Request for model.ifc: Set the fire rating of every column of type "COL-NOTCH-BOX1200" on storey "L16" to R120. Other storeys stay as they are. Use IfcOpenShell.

First a look at what the model holds.

```python
import ifcopenshell
import ifcopenshell.util.element

model = ifcopenshell.open("model.ifc")
print(model.schema)
storey = next(s for s in model.by_type("IfcBuildingStorey") if s.Name == "L16")
columns = [e for e in ifcopenshell.util.element.get_decomposition(storey) if e.is_a("IfcColumn")]
seen = {}
for e in columns:
    element_type = ifcopenshell.util.element.get_type(e)
    key = (element_type.Name if element_type != e and element_type else None, ifcopenshell.util.element.get_pset(e, "Pset_ColumnCommon", "FireRating"))
    seen[key] = seen.get(key, 0) + 1
for (name, value), count in sorted(seen.items(), key=str):
    print(count, "x", name, "|", value)
```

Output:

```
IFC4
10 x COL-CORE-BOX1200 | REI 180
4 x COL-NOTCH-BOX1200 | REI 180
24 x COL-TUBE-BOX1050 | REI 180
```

```python
import ifcopenshell
import ifcopenshell.api.pset
import ifcopenshell.util.element

model = ifcopenshell.open("model.ifc")

storey = next(s for s in model.by_type("IfcBuildingStorey") if s.Name == "L16")
columns = [e for e in ifcopenshell.util.element.get_decomposition(storey) if e.is_a("IfcColumn")]

count = 0
for e in columns:
    element_type = ifcopenshell.util.element.get_type(e)
    if element_type in (None, e) or element_type.Name != "COL-NOTCH-BOX1200":
        continue
    found = ifcopenshell.util.element.get_pset(e, "Pset_ColumnCommon", should_inherit=False)
    if found:
        pset = model.by_id(found["id"])
        if len(ifcopenshell.util.element.get_elements_by_pset(pset)) > 1:
            pset = ifcopenshell.api.pset.unshare_pset(model, products=[e], pset=pset)[0]
    else:
        pset = ifcopenshell.api.pset.add_pset(model, product=e, name="Pset_ColumnCommon")
    ifcopenshell.api.pset.edit_pset(model, pset=pset, properties={"FireRating": "R120"})
    count += 1

print(count, "columns updated")

model.write("model_updated.ifc")
```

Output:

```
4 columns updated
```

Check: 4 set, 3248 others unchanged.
